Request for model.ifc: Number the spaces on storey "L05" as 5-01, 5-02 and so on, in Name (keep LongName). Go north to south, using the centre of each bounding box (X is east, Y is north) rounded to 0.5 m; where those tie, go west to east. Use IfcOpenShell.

First a look at what the model holds.

```python
import ifcopenshell
import ifcopenshell.util.element
import ifcopenshell.util.placement

model = ifcopenshell.open("model.ifc")
print(model.schema)
storey = next(s for s in model.by_type("IfcBuildingStorey") if s.Name == "L05")
spaces = [e for e in ifcopenshell.util.element.get_decomposition(storey) if e.is_a("IfcSpace")]
for e in sorted(spaces, key=lambda e: e.id()):
    origin = ifcopenshell.util.placement.get_local_placement(e.ObjectPlacement)[:3, 3]
    print(e.id(), e.Name, e.LongName, origin.round(2) + 0.0, sep=" | ")
```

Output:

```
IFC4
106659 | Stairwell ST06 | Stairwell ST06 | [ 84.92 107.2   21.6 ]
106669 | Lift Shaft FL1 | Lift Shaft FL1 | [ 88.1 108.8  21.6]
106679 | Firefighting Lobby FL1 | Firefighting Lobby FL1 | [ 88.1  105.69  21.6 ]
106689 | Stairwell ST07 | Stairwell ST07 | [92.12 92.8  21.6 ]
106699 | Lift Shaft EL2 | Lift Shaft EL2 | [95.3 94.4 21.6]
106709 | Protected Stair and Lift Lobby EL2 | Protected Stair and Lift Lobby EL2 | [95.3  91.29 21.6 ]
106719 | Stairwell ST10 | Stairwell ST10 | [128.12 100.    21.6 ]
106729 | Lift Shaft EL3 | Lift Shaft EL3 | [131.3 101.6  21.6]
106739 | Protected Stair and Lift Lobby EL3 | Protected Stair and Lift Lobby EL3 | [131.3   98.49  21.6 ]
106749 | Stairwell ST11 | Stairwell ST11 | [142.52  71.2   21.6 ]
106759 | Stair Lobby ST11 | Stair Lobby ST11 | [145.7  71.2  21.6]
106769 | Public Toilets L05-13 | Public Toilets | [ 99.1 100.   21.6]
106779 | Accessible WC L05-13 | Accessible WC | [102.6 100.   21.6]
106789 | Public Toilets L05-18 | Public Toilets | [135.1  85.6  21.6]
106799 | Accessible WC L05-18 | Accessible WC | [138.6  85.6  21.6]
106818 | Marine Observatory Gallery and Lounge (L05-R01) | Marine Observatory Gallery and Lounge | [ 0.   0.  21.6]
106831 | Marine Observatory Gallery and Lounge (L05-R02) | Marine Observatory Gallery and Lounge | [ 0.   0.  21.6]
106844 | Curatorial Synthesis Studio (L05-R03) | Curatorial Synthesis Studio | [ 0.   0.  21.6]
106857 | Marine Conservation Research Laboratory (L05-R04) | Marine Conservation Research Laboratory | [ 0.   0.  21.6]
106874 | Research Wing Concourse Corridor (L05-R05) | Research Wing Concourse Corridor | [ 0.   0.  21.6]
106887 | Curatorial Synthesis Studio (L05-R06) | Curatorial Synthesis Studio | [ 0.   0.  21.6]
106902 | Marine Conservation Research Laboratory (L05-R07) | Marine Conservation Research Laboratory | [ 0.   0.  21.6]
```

```python
import ifcopenshell
import ifcopenshell.geom
import ifcopenshell.util.element
import ifcopenshell.util.shape

model = ifcopenshell.open("model.ifc")
settings = ifcopenshell.geom.settings()
settings.set("use-world-coords", True)


def centre(element):
    shape = ifcopenshell.geom.create_shape(settings, element)
    return ifcopenshell.util.shape.get_bbox_centroid(shape.geometry)


storey = next(s for s in model.by_type("IfcBuildingStorey") if s.Name == "L05")
spaces = [e for e in ifcopenshell.util.element.get_decomposition(storey) if e.is_a("IfcSpace")]

# Insertion points can sit at a corner or the storey origin, so sort by the geometry (in metres).
centres = {e: centre(e) for e in spaces}
spaces.sort(key=lambda e: (-round(centres[e][1] / 0.5), centres[e][0]))

for i, e in enumerate(spaces, start=1):
    number = f"5-{i:02d}"
    e.Name = number
    print(e.id(), number)

model.write("model_rev.ifc")
```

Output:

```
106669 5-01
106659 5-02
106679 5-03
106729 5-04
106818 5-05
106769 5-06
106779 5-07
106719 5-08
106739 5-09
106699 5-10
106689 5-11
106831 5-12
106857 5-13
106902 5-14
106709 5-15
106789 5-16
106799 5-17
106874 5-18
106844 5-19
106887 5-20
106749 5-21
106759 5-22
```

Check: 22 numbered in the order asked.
